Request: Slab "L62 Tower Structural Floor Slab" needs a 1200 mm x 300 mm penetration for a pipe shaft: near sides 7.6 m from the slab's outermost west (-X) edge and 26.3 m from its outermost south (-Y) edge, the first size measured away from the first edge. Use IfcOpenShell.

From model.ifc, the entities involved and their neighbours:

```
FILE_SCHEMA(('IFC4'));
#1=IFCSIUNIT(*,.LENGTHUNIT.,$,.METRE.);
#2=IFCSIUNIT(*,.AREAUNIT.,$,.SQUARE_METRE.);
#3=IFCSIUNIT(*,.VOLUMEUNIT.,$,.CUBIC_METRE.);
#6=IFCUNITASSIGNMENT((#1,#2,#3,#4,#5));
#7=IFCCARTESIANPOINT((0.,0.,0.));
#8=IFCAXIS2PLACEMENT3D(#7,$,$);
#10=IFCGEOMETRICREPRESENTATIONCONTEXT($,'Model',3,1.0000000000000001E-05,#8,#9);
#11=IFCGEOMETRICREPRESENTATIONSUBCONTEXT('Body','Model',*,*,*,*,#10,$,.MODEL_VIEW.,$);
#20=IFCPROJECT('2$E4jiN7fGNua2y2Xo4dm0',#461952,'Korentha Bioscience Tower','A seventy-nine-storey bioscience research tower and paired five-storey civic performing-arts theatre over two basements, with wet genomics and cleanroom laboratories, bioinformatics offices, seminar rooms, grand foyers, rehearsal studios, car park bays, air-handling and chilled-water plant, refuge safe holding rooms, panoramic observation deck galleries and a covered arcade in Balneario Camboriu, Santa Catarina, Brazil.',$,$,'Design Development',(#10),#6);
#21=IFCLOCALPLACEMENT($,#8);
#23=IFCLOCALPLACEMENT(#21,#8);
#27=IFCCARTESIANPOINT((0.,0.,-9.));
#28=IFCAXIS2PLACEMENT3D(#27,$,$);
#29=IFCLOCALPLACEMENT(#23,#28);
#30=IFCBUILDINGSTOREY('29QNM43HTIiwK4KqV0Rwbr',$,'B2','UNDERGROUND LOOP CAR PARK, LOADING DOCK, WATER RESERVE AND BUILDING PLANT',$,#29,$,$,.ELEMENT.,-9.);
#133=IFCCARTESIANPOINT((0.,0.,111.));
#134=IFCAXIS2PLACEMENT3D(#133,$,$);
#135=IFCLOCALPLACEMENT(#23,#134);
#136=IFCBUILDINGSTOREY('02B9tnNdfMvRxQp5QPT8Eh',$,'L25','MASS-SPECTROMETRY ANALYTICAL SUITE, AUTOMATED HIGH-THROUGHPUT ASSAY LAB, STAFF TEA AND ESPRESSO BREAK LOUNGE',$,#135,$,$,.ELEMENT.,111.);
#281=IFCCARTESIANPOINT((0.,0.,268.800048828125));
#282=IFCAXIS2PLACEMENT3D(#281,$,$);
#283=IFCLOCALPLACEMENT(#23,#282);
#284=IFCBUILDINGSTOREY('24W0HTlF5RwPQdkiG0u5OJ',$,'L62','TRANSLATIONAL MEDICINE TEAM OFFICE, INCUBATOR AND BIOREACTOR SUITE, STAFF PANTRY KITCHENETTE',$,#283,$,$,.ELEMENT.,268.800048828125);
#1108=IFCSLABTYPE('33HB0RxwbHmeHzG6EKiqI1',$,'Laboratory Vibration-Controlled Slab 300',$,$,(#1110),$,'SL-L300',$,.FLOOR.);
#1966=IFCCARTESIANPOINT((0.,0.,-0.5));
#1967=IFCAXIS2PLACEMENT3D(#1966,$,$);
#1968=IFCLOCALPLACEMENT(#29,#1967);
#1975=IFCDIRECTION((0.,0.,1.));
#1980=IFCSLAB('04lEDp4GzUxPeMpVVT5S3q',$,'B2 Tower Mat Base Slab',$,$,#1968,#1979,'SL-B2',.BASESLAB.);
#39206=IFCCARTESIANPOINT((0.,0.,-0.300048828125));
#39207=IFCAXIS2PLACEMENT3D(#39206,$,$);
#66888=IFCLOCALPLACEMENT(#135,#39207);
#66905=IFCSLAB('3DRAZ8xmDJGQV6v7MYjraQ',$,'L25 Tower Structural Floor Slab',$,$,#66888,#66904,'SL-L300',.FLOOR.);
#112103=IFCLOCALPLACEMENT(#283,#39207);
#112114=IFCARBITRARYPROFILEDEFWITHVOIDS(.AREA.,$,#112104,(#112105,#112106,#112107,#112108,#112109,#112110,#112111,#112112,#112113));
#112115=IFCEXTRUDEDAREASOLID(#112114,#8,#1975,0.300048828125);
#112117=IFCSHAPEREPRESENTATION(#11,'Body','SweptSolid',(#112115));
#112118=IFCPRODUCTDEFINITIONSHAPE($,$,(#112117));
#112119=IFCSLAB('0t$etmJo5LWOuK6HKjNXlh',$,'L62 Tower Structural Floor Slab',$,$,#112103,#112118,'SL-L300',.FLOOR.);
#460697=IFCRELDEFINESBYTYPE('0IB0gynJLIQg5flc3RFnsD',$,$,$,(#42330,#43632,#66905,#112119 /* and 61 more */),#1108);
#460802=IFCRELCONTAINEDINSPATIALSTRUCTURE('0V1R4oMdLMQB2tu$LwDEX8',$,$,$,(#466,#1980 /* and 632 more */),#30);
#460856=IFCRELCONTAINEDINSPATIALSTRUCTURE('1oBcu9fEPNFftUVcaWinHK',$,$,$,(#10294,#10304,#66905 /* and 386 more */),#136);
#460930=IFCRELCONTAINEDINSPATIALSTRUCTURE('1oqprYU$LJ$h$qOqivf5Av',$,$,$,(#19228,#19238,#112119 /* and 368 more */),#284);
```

```python
import numpy as np
import ifcopenshell
import ifcopenshell.api.feature
import ifcopenshell.api.geometry
import ifcopenshell.api.root
import ifcopenshell.geom
import ifcopenshell.util.placement
import ifcopenshell.util.representation
import ifcopenshell.util.shape
import ifcopenshell.util.unit

model = ifcopenshell.open("model.ifc")
unit_scale = ifcopenshell.util.unit.calculate_unit_scale(model)
settings = ifcopenshell.geom.settings()


def volume(element):
    """Net volume in cubic metres, openings subtracted."""
    shape = ifcopenshell.geom.create_shape(settings, element)
    return ifcopenshell.util.shape.get_volume(shape.geometry)


slab = model.by_id(112119)
before = volume(slab)

# Extent in the slab's own axes, in metres. The edges named are its -X and -Y sides.
slab_shape = ifcopenshell.geom.create_shape(settings, slab)
vertices = ifcopenshell.util.shape.get_vertices(slab_shape.geometry)
x_min, y_min, bottom = vertices.min(axis=0)
top = vertices[:, 2].max()

opening = ifcopenshell.api.root.create_entity(model, ifc_class="IfcOpeningElement", name="Pipe shaft opening", predefined_type="OPENING")
context = ifcopenshell.util.representation.get_context(model, "Model", "Body", "MODEL_VIEW")
width, depth = 1.2, 0.3
outline = [(0.0, 0.0), (width, 0.0), (width, depth), (0.0, depth), (0.0, 0.0)]
# Overshoot both faces by 50 mm so the cut is clean.
shape = ifcopenshell.api.geometry.add_slab_representation(
    model, context=context, depth=top - bottom + 0.1, polyline=outline
)
ifcopenshell.api.geometry.assign_representation(model, product=opening, representation=shape)

matrix = ifcopenshell.util.placement.get_local_placement(slab.ObjectPlacement)
matrix[:, 3] = matrix @ np.append(np.array([x_min + 7.6, y_min + 26.3, bottom - 0.05]) / unit_scale, 1.0)
ifcopenshell.api.geometry.edit_object_placement(model, product=opening, matrix=matrix, is_si=False)
ifcopenshell.api.feature.add_feature(model, feature=opening, element=slab)

after = volume(slab)

print(f"slab volume {before:.3f} -> {after:.3f} m3")

model.write("model_rev.ifc")
```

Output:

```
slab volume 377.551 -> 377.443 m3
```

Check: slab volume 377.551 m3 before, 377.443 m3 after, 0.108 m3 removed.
